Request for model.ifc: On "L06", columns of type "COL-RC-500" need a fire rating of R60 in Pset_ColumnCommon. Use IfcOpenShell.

First a look at what the model holds.

```python
import ifcopenshell
import ifcopenshell.util.element

model = ifcopenshell.open("model.ifc")
print(model.schema)
storey = next(s for s in model.by_type("IfcBuildingStorey") if s.Name == "L06")
columns = [e for e in ifcopenshell.util.element.get_decomposition(storey) if e.is_a("IfcColumn")]
seen = {}
for e in columns:
    element_type = ifcopenshell.util.element.get_type(e)
    key = (element_type.Name if element_type != e and element_type else None, ifcopenshell.util.element.get_pset(e, "Pset_ColumnCommon", "FireRating"))
    seen[key] = seen.get(key, 0) + 1
for (name, value), count in sorted(seen.items(), key=str):
    print(count, "x", name, "|", value)
```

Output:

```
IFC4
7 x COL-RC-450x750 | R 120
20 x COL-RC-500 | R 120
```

```python
import ifcopenshell
import ifcopenshell.api.pset
import ifcopenshell.util.element

model = ifcopenshell.open("model.ifc")

storey = next(s for s in model.by_type("IfcBuildingStorey") if s.Name == "L06")
columns = [e for e in ifcopenshell.util.element.get_decomposition(storey) if e.is_a("IfcColumn")]

count = 0
for e in columns:
    element_type = ifcopenshell.util.element.get_type(e)
    if element_type in (None, e) or element_type.Name != "COL-RC-500":
        continue
    # add_pset returns the element's existing set when there is one.
    pset = ifcopenshell.api.pset.add_pset(model, product=e, name="Pset_ColumnCommon")
    ifcopenshell.api.pset.edit_pset(model, pset=pset, properties={"FireRating": "R60"})
    count += 1

print(count, "columns updated")

model.write("model_rev.ifc")
```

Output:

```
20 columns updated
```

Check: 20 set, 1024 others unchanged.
